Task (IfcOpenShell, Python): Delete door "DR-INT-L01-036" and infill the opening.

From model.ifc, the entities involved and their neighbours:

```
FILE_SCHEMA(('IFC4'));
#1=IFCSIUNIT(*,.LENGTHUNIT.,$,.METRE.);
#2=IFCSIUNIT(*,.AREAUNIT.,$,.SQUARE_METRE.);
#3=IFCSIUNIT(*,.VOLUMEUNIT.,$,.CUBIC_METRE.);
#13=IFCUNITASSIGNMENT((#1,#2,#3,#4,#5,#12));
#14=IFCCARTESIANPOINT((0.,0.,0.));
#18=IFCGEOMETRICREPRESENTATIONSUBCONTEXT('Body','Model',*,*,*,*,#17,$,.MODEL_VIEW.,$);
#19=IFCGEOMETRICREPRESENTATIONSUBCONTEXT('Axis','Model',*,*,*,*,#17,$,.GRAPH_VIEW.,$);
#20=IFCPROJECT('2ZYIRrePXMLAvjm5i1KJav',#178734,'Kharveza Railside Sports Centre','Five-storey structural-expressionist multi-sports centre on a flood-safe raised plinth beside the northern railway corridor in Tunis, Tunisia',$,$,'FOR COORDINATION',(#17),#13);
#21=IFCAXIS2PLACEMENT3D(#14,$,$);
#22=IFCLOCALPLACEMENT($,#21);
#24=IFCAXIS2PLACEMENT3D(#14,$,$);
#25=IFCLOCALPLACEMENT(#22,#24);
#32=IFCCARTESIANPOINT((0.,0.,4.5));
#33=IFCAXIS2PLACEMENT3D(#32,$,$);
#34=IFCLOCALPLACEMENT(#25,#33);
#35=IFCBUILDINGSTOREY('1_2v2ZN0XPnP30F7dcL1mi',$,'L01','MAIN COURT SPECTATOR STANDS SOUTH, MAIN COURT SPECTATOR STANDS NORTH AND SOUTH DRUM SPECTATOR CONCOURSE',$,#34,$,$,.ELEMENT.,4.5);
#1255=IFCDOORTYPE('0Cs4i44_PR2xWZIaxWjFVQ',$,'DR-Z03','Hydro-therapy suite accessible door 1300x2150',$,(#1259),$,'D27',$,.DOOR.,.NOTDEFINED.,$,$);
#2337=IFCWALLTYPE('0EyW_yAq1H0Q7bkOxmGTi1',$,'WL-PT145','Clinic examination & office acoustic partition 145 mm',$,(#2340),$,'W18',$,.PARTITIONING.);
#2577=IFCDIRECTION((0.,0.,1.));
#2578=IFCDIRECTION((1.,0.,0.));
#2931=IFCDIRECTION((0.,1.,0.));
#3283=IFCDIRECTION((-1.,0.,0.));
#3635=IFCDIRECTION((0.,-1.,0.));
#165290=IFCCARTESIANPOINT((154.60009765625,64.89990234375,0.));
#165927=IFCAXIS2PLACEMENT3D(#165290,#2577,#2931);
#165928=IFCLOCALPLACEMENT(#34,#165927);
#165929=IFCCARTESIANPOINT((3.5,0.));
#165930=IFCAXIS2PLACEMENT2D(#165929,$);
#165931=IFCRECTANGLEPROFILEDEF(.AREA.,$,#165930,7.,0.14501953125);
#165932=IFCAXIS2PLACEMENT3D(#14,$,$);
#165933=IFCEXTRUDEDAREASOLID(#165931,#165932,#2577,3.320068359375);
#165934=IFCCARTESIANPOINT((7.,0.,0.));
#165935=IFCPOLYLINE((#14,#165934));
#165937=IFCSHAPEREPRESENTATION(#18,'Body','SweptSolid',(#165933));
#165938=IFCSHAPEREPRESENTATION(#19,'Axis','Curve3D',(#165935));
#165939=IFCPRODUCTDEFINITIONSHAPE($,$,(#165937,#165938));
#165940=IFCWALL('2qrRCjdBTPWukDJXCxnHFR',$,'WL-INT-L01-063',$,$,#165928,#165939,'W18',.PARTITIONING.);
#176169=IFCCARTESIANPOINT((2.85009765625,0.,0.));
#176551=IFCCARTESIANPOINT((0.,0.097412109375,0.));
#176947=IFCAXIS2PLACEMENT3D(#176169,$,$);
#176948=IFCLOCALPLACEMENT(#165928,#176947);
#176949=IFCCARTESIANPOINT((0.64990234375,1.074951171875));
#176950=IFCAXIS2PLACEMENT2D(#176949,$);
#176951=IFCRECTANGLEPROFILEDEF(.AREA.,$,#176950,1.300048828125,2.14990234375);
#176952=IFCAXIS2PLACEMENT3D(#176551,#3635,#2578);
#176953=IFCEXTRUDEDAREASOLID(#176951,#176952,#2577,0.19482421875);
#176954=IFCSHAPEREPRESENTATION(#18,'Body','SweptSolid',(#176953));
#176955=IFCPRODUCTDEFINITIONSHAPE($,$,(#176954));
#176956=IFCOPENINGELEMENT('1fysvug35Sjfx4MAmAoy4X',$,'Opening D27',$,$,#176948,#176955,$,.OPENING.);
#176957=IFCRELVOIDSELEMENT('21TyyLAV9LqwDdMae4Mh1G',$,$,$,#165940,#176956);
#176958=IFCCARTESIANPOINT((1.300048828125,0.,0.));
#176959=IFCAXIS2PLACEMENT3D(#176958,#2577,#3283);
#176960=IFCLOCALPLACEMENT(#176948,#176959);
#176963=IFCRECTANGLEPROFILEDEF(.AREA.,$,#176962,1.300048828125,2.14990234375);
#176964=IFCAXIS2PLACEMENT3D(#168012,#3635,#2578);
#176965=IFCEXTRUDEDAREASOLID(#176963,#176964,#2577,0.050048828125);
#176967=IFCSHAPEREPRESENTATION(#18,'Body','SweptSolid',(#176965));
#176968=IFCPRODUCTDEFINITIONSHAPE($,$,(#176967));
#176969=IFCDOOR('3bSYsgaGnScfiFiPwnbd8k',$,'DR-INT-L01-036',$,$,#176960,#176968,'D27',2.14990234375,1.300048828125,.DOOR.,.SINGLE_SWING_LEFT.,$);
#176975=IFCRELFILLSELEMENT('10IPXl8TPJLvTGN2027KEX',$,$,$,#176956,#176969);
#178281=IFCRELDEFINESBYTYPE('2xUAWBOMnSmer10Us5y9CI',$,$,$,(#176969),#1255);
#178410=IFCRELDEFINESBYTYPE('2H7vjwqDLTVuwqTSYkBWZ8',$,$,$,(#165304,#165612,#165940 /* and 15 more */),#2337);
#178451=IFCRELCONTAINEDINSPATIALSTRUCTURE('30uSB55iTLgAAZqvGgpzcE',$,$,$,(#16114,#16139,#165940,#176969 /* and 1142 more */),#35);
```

```python
import ifcopenshell
import ifcopenshell.api.feature
import ifcopenshell.api.root
import ifcopenshell.geom
import ifcopenshell.util.shape

model = ifcopenshell.open("model.ifc")
settings = ifcopenshell.geom.settings()


def volume(element):
    """Net volume in cubic metres, openings subtracted."""
    shape = ifcopenshell.geom.create_shape(settings, element)
    return ifcopenshell.util.shape.get_volume(shape.geometry)


door = model.by_id(176969)
opening = door.FillsVoids[0].RelatingOpeningElement
wall = opening.VoidsElements[0].RelatingBuildingElement
before = volume(wall)

ifcopenshell.api.root.remove_product(model, product=door)
ifcopenshell.api.feature.remove_feature(model, feature=opening)

after = volume(wall)

print(f"wall volume {before:.3f} -> {after:.3f} m3")

model.write("model-out.ifc")
```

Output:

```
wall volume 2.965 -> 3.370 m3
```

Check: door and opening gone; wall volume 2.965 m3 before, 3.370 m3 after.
